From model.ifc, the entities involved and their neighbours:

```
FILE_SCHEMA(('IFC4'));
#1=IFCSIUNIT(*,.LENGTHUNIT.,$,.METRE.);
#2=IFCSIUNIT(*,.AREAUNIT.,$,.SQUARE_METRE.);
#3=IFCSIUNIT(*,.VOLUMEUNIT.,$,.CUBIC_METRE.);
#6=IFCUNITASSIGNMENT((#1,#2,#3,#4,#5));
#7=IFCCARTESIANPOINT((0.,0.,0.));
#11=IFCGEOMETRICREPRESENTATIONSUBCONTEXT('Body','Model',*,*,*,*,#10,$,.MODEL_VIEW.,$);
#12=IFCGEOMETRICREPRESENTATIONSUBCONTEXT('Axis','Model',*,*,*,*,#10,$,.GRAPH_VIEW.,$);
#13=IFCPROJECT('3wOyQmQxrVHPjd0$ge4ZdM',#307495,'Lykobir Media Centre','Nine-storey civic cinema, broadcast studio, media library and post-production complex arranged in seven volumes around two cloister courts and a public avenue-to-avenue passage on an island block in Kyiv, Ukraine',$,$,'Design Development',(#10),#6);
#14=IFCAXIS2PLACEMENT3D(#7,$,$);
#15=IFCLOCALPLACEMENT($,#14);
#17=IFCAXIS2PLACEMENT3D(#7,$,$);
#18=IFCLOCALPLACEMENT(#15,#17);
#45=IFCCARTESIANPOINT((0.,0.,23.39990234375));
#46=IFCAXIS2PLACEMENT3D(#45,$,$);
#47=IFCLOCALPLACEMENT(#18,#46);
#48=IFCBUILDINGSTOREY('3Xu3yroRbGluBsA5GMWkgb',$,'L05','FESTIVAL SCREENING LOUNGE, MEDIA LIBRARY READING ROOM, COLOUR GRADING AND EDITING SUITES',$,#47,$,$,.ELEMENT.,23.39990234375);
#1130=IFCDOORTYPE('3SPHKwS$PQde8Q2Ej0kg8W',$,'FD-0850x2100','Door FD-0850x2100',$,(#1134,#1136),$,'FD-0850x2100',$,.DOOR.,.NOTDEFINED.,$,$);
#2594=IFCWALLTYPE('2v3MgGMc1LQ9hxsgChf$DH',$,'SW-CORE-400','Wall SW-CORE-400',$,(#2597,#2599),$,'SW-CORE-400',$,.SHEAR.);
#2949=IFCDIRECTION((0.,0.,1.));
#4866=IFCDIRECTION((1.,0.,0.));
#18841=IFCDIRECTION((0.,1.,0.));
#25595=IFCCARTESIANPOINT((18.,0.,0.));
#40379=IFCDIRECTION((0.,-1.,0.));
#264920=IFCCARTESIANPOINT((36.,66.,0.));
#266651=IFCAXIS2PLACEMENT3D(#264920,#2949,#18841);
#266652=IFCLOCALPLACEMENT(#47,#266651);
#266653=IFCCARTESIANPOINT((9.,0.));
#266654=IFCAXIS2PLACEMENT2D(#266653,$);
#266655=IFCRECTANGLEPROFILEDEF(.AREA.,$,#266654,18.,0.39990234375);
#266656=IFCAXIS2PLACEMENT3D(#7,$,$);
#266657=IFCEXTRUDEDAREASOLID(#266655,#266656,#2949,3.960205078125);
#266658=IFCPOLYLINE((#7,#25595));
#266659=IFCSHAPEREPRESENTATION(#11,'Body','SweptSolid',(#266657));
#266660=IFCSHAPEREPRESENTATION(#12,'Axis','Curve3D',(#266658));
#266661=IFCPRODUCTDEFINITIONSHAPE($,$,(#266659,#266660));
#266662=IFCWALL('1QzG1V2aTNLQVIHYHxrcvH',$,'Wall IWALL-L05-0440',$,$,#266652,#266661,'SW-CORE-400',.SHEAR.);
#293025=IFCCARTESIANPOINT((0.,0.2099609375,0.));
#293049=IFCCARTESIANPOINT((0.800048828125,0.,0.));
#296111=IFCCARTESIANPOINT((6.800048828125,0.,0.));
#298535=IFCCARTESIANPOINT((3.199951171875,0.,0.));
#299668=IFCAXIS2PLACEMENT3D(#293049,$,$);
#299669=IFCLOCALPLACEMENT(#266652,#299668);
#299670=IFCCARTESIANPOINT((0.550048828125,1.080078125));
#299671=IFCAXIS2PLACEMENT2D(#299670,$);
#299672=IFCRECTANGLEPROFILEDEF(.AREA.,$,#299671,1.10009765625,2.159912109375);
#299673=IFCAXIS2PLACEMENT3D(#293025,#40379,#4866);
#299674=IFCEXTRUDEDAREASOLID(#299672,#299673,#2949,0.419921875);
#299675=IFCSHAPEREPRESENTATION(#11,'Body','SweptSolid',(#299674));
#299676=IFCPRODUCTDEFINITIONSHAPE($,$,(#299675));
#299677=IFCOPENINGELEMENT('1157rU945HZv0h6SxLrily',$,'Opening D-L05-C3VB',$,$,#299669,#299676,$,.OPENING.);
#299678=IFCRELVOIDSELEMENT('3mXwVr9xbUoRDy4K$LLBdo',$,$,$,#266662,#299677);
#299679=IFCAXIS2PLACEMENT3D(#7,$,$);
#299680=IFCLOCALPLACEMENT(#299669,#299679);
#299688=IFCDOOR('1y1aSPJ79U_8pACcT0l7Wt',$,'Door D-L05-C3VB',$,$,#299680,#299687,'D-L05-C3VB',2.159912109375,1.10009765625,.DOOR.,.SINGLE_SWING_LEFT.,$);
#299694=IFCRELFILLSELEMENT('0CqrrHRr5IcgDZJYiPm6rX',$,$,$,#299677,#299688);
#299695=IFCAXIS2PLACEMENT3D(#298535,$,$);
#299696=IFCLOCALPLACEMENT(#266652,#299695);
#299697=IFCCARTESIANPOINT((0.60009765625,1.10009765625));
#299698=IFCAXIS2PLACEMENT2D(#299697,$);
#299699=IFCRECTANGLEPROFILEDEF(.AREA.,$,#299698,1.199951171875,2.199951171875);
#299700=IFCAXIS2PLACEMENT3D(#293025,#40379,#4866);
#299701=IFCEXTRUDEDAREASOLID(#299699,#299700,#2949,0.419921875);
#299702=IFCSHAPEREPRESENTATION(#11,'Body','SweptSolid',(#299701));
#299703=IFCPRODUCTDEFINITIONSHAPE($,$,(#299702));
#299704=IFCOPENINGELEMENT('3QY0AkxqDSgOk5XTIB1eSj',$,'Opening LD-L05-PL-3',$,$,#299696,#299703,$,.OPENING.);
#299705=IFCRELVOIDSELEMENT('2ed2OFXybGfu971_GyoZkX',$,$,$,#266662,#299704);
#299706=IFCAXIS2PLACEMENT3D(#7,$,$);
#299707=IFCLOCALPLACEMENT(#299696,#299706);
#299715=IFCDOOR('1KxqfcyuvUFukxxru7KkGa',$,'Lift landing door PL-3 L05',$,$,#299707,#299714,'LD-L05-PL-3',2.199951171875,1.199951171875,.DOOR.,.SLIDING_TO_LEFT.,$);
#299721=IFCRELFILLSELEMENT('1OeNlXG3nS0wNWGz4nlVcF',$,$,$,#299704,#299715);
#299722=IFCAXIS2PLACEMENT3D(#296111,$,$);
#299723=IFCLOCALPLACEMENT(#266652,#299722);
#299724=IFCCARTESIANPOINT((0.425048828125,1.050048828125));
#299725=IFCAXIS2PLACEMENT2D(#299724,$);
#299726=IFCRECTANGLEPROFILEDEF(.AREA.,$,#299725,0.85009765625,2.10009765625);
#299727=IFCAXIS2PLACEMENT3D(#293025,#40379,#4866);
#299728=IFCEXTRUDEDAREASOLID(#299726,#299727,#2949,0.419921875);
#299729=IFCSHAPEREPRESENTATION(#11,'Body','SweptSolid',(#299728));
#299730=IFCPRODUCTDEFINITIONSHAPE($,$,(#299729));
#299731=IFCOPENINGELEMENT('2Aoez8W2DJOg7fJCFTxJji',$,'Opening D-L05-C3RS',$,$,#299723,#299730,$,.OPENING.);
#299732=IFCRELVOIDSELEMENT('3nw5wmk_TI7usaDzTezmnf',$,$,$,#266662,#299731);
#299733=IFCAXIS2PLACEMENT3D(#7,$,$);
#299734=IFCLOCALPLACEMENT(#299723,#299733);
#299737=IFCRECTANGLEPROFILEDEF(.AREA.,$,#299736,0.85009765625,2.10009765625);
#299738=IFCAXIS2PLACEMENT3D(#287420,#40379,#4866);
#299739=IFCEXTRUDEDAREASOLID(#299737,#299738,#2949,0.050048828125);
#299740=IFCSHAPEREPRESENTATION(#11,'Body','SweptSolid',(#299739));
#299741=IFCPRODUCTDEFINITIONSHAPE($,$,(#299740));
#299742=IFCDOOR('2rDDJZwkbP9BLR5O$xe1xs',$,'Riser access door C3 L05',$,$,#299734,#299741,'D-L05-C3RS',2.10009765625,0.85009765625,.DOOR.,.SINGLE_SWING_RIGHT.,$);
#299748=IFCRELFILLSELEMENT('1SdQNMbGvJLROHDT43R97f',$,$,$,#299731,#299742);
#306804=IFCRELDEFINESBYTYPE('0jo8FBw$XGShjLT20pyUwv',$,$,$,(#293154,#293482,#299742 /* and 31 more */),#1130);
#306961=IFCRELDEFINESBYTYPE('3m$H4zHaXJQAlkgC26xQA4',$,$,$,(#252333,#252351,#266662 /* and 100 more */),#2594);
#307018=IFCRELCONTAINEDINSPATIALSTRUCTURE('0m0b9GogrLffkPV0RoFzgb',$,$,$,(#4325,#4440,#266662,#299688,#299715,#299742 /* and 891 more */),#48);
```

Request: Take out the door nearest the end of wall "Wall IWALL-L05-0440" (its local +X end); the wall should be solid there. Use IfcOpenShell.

```python
import ifcopenshell
import ifcopenshell.api.feature
import ifcopenshell.api.root
import ifcopenshell.geom
import ifcopenshell.util.shape

model = ifcopenshell.open("model.ifc")
settings = ifcopenshell.geom.settings()


def volume(element):
    """Net volume in cubic metres, openings subtracted."""
    shape = ifcopenshell.geom.create_shape(settings, element)
    return ifcopenshell.util.shape.get_volume(shape.geometry)


door = model.by_guid("2rDDJZwkbP9BLR5O$xe1xs")
opening = door.FillsVoids[0].RelatingOpeningElement
wall = opening.VoidsElements[0].RelatingBuildingElement
before = volume(wall)

ifcopenshell.api.root.remove_product(model, product=door)
ifcopenshell.api.feature.remove_feature(model, feature=opening)

after = volume(wall)

print(f"wall volume {before:.3f} -> {after:.3f} m3")

model.write("model_v2.ifc")
```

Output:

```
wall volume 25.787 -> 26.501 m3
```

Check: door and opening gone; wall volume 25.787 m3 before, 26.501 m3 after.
